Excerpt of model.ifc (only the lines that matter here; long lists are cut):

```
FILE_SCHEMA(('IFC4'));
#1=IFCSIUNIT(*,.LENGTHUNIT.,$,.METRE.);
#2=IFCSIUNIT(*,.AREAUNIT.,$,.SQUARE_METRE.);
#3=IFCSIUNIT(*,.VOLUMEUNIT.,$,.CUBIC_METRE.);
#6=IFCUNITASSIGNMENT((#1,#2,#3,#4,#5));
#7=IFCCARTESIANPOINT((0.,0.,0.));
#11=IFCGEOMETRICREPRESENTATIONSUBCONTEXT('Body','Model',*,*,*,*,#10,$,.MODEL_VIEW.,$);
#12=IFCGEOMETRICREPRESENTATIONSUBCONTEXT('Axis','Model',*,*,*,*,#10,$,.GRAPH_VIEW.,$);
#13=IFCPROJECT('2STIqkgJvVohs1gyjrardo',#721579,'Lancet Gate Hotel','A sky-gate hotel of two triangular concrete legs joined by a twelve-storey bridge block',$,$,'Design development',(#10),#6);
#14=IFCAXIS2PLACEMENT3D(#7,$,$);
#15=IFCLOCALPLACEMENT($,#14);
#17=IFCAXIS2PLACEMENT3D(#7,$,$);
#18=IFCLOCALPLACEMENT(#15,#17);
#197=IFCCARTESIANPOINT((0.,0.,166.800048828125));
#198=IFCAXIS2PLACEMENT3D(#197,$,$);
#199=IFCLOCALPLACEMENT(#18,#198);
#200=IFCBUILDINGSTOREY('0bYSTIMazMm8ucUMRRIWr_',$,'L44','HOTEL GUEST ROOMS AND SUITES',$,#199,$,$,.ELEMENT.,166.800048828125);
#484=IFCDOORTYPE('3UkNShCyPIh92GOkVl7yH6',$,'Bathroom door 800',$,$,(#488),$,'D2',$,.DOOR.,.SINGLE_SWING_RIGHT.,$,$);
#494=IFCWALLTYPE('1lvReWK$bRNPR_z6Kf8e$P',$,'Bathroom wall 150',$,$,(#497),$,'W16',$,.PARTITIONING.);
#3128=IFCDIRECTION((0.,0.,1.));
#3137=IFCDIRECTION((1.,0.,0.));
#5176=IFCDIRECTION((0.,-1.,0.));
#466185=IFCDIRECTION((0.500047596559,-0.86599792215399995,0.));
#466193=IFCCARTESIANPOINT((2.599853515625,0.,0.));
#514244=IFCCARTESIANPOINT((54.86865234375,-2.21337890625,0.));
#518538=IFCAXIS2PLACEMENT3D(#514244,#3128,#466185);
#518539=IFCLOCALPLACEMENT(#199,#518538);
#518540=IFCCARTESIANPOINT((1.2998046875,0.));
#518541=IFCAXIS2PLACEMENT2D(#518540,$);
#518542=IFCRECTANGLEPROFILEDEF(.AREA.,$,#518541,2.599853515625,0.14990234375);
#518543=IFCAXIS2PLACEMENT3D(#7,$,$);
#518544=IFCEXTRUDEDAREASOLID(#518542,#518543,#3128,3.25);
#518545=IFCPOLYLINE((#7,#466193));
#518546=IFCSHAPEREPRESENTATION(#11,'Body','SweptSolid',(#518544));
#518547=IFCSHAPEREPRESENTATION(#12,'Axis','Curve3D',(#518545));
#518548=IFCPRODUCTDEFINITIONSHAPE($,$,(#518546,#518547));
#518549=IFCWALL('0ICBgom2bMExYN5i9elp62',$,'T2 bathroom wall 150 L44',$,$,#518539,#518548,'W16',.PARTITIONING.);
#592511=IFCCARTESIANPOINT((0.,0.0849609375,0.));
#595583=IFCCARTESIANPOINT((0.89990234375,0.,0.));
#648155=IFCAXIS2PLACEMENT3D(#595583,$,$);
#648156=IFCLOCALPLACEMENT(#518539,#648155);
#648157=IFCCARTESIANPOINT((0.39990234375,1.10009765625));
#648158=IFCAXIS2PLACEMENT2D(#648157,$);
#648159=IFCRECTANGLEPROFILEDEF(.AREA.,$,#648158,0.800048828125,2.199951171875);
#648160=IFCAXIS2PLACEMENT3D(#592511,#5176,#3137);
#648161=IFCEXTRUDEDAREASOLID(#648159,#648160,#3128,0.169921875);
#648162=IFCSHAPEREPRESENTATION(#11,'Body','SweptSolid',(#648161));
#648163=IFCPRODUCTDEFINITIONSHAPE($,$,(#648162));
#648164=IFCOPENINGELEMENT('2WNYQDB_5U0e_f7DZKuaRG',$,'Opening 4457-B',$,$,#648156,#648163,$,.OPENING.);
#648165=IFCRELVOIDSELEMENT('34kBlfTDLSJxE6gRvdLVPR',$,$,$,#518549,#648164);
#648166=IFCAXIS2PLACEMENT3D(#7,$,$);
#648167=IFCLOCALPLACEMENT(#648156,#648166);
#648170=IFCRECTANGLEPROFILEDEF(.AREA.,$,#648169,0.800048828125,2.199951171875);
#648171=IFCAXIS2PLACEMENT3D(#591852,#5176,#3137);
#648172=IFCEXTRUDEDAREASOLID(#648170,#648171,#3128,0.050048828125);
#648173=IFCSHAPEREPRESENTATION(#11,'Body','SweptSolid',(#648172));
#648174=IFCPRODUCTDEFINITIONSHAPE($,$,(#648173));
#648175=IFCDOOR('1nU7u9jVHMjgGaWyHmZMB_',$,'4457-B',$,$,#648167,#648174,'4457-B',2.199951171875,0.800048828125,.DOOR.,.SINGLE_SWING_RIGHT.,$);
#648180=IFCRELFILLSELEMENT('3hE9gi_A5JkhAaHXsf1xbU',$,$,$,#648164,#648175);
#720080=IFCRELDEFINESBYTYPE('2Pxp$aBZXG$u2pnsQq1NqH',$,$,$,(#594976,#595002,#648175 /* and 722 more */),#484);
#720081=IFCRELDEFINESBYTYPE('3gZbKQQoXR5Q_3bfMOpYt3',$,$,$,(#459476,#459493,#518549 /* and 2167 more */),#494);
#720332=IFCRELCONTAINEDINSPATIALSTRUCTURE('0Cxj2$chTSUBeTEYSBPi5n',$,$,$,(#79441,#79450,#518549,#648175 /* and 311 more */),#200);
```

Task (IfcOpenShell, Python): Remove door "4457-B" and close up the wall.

```python
import ifcopenshell
import ifcopenshell.api.feature
import ifcopenshell.api.root
import ifcopenshell.geom
import ifcopenshell.util.shape

model = ifcopenshell.open("model.ifc")
settings = ifcopenshell.geom.settings()


def volume(element):
    """Net volume in cubic metres, openings subtracted."""
    shape = ifcopenshell.geom.create_shape(settings, element)
    return ifcopenshell.util.shape.get_volume(shape.geometry)


door = model.by_id(648175)
opening = door.FillsVoids[0].RelatingOpeningElement
wall = opening.VoidsElements[0].RelatingBuildingElement
before = volume(wall)

ifcopenshell.api.root.remove_product(model, product=door)
ifcopenshell.api.feature.remove_feature(model, feature=opening)

after = volume(wall)

print(f"wall volume {before:.3f} -> {after:.3f} m3")

model.write("model-out.ifc")
```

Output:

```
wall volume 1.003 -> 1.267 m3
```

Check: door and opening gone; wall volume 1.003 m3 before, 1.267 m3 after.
